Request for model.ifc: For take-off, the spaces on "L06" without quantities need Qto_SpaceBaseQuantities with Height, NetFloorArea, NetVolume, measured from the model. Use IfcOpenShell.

First a look at what the model holds.

```python
import ifcopenshell
import ifcopenshell.util.element
import ifcopenshell.util.unit

model = ifcopenshell.open("model.ifc")
print(model.schema)
for unit_type in ("LENGTHUNIT", "AREAUNIT", "VOLUMEUNIT"):
    print(unit_type, ifcopenshell.util.unit.calculate_unit_scale(model, unit_type))
storey = next(s for s in model.by_type("IfcBuildingStorey") if s.Name == "L06")
spaces = [e for e in ifcopenshell.util.element.get_decomposition(storey) if e.is_a("IfcSpace")]
for e in sorted(spaces, key=lambda e: e.id()):
    print(e.id(), e.is_a(), e.Name, list(ifcopenshell.util.element.get_psets(e, qtos_only=True)), sep=" | ")
```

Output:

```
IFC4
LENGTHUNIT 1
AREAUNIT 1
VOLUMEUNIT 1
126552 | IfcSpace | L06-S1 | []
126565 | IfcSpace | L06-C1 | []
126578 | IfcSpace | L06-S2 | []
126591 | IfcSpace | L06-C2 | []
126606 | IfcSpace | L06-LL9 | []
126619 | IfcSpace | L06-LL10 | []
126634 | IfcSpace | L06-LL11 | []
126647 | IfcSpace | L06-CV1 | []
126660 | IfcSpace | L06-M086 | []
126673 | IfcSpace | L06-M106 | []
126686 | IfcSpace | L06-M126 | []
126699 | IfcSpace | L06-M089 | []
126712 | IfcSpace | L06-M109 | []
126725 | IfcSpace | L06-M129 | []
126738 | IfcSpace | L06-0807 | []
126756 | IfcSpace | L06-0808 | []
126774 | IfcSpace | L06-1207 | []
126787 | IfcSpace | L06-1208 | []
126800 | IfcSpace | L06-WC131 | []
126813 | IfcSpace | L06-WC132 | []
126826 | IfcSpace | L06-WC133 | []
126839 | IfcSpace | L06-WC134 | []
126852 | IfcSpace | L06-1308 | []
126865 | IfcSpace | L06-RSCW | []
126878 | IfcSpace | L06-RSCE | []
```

```python
import ifcopenshell
import ifcopenshell.api.pset
import ifcopenshell.geom
import ifcopenshell.util.element
import ifcopenshell.util.shape
import ifcopenshell.util.unit

model = ifcopenshell.open("model.ifc")
unit_scale = ifcopenshell.util.unit.calculate_unit_scale(model)
area_scale = ifcopenshell.util.unit.calculate_unit_scale(model, "AREAUNIT")
volume_scale = ifcopenshell.util.unit.calculate_unit_scale(model, "VOLUMEUNIT")
settings = ifcopenshell.geom.settings()

storey = next(s for s in model.by_type("IfcBuildingStorey") if s.Name == "L06")
spaces = [e for e in ifcopenshell.util.element.get_decomposition(storey) if e.is_a("IfcSpace")]

for e in sorted(spaces, key=lambda e: e.id()):
    if ifcopenshell.util.element.get_psets(e, qtos_only=True, should_inherit=False):
        continue
    # Geometry comes back in metres, in the element's own axes.
    shape = ifcopenshell.geom.create_shape(settings, e)
    values = {
        "Height": ifcopenshell.util.shape.get_z(shape.geometry) / unit_scale,
        "NetFloorArea": ifcopenshell.util.shape.get_footprint_area(shape.geometry) / area_scale,
        "NetVolume": ifcopenshell.util.shape.get_volume(shape.geometry) / volume_scale,
    }
    qto = ifcopenshell.api.pset.add_qto(model, product=e, name="Qto_SpaceBaseQuantities")
    ifcopenshell.api.pset.edit_qto(model, qto=qto, properties=values)
    print(e.id(), {k: round(v, 3) for k, v in values.items()})

model.write("model-out.ifc")
```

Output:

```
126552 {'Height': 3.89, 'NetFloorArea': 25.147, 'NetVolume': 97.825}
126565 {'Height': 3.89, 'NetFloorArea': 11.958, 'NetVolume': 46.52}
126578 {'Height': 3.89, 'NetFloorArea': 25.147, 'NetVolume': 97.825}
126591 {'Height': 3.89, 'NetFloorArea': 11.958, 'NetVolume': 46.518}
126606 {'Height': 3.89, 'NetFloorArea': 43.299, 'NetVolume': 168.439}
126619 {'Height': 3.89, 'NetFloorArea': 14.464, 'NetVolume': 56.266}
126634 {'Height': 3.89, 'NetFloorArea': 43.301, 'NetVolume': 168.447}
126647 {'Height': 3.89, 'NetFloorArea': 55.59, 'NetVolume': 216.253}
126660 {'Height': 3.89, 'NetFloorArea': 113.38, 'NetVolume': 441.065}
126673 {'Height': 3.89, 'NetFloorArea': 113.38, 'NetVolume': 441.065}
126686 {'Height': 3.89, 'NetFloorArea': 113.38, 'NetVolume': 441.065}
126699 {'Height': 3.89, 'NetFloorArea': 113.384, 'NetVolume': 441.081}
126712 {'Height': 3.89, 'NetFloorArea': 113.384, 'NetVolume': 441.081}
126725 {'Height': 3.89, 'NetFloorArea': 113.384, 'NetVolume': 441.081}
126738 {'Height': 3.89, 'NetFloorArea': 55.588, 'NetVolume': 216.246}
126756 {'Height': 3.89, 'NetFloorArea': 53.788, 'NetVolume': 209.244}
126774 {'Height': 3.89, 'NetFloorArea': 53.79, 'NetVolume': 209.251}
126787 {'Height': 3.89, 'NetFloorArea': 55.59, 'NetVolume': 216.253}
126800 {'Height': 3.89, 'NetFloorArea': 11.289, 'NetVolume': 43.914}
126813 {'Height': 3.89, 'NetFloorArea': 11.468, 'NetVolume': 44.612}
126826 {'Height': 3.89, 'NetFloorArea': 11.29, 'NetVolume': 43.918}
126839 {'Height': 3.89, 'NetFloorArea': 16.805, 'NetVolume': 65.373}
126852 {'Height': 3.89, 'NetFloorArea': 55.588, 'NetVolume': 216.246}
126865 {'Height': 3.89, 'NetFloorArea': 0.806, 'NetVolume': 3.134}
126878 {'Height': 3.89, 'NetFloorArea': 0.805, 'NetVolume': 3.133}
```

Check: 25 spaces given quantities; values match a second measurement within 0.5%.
